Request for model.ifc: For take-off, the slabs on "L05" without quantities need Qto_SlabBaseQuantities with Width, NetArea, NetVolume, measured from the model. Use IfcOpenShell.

First a look at what the model holds.

```python
import ifcopenshell
import ifcopenshell.util.element
import ifcopenshell.util.unit

model = ifcopenshell.open("model.ifc")
print(model.schema)
for unit_type in ("LENGTHUNIT", "AREAUNIT", "VOLUMEUNIT"):
    print(unit_type, ifcopenshell.util.unit.calculate_unit_scale(model, unit_type))
storey = next(s for s in model.by_type("IfcBuildingStorey") if s.Name == "L05")
slabs = [e for e in ifcopenshell.util.element.get_decomposition(storey) if e.is_a("IfcSlab")]
for e in sorted(slabs, key=lambda e: e.id()):
    print(e.id(), e.is_a(), e.Name, list(ifcopenshell.util.element.get_psets(e, qtos_only=True)), sep=" | ")
```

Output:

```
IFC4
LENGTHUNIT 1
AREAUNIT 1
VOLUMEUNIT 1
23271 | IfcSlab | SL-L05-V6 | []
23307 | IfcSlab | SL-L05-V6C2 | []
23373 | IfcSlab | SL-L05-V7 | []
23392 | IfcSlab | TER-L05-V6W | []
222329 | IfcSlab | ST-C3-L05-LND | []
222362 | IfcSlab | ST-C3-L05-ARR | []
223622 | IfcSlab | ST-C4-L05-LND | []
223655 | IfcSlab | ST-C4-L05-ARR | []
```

```python
import ifcopenshell
import ifcopenshell.api.pset
import ifcopenshell.geom
import ifcopenshell.util.element
import ifcopenshell.util.shape
import ifcopenshell.util.unit

model = ifcopenshell.open("model.ifc")
unit_scale = ifcopenshell.util.unit.calculate_unit_scale(model)
area_scale = ifcopenshell.util.unit.calculate_unit_scale(model, "AREAUNIT")
volume_scale = ifcopenshell.util.unit.calculate_unit_scale(model, "VOLUMEUNIT")
settings = ifcopenshell.geom.settings()

storey = next(s for s in model.by_type("IfcBuildingStorey") if s.Name == "L05")
slabs = [e for e in ifcopenshell.util.element.get_decomposition(storey) if e.is_a("IfcSlab")]

for e in sorted(slabs, key=lambda e: e.id()):
    if ifcopenshell.util.element.get_psets(e, qtos_only=True, should_inherit=False):
        continue
    # Geometry comes back in metres, in the element's own axes.
    shape = ifcopenshell.geom.create_shape(settings, e)
    values = {
        "Width": ifcopenshell.util.shape.get_z(shape.geometry) / unit_scale,
        "NetArea": ifcopenshell.util.shape.get_footprint_area(shape.geometry) / area_scale,
        "NetVolume": ifcopenshell.util.shape.get_volume(shape.geometry) / volume_scale,
    }
    qto = ifcopenshell.api.pset.add_qto(model, product=e, name="Qto_SlabBaseQuantities")
    ifcopenshell.api.pset.edit_qto(model, qto=qto, properties=values)
    print(e.id(), {k: round(v, 3) for k, v in values.items()})

model.write("model_rev.ifc")
```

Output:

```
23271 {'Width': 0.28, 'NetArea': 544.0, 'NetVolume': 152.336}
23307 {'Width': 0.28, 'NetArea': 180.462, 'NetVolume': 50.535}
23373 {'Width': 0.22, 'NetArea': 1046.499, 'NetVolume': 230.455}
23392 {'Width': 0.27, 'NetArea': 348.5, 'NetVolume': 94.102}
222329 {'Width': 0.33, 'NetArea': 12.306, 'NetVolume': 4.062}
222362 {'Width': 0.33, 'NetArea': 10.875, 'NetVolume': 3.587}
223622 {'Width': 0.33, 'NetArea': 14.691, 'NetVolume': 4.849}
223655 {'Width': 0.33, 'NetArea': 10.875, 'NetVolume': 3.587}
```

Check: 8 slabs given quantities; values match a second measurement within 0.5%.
